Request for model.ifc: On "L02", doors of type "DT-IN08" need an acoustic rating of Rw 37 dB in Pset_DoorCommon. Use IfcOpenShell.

First a look at what the model holds.

```python
import ifcopenshell
import ifcopenshell.util.element

model = ifcopenshell.open("model.ifc")
print(model.schema)
storey = next(s for s in model.by_type("IfcBuildingStorey") if s.Name == "L02")
doors = [e for e in ifcopenshell.util.element.get_decomposition(storey) if e.is_a("IfcDoor")]
seen = {}
for e in doors:
    element_type = ifcopenshell.util.element.get_type(e)
    key = (element_type.Name if element_type != e and element_type else None, ifcopenshell.util.element.get_pset(e, "Pset_DoorCommon", "AcousticRating"))
    seen[key] = seen.get(key, 0) + 1
for (name, value), count in sorted(seen.items(), key=str):
    print(count, "x", name, "|", value)
```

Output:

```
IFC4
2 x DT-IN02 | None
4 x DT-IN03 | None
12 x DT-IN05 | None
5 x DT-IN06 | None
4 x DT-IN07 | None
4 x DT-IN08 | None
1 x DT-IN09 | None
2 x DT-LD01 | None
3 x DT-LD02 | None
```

```python
import ifcopenshell
import ifcopenshell.api.pset
import ifcopenshell.util.element

model = ifcopenshell.open("model.ifc")

storey = next(s for s in model.by_type("IfcBuildingStorey") if s.Name == "L02")
doors = [e for e in ifcopenshell.util.element.get_decomposition(storey) if e.is_a("IfcDoor")]

count = 0
for e in doors:
    element_type = ifcopenshell.util.element.get_type(e)
    if element_type in (None, e) or element_type.Name != "DT-IN08":
        continue
    # add_pset returns the element's existing set when there is one.
    pset = ifcopenshell.api.pset.add_pset(model, product=e, name="Pset_DoorCommon")
    ifcopenshell.api.pset.edit_pset(model, pset=pset, properties={"AcousticRating": "Rw 37 dB"})
    count += 1

print(count, "doors updated")

model.write("model_edited.ifc")
```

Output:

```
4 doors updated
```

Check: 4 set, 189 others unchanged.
